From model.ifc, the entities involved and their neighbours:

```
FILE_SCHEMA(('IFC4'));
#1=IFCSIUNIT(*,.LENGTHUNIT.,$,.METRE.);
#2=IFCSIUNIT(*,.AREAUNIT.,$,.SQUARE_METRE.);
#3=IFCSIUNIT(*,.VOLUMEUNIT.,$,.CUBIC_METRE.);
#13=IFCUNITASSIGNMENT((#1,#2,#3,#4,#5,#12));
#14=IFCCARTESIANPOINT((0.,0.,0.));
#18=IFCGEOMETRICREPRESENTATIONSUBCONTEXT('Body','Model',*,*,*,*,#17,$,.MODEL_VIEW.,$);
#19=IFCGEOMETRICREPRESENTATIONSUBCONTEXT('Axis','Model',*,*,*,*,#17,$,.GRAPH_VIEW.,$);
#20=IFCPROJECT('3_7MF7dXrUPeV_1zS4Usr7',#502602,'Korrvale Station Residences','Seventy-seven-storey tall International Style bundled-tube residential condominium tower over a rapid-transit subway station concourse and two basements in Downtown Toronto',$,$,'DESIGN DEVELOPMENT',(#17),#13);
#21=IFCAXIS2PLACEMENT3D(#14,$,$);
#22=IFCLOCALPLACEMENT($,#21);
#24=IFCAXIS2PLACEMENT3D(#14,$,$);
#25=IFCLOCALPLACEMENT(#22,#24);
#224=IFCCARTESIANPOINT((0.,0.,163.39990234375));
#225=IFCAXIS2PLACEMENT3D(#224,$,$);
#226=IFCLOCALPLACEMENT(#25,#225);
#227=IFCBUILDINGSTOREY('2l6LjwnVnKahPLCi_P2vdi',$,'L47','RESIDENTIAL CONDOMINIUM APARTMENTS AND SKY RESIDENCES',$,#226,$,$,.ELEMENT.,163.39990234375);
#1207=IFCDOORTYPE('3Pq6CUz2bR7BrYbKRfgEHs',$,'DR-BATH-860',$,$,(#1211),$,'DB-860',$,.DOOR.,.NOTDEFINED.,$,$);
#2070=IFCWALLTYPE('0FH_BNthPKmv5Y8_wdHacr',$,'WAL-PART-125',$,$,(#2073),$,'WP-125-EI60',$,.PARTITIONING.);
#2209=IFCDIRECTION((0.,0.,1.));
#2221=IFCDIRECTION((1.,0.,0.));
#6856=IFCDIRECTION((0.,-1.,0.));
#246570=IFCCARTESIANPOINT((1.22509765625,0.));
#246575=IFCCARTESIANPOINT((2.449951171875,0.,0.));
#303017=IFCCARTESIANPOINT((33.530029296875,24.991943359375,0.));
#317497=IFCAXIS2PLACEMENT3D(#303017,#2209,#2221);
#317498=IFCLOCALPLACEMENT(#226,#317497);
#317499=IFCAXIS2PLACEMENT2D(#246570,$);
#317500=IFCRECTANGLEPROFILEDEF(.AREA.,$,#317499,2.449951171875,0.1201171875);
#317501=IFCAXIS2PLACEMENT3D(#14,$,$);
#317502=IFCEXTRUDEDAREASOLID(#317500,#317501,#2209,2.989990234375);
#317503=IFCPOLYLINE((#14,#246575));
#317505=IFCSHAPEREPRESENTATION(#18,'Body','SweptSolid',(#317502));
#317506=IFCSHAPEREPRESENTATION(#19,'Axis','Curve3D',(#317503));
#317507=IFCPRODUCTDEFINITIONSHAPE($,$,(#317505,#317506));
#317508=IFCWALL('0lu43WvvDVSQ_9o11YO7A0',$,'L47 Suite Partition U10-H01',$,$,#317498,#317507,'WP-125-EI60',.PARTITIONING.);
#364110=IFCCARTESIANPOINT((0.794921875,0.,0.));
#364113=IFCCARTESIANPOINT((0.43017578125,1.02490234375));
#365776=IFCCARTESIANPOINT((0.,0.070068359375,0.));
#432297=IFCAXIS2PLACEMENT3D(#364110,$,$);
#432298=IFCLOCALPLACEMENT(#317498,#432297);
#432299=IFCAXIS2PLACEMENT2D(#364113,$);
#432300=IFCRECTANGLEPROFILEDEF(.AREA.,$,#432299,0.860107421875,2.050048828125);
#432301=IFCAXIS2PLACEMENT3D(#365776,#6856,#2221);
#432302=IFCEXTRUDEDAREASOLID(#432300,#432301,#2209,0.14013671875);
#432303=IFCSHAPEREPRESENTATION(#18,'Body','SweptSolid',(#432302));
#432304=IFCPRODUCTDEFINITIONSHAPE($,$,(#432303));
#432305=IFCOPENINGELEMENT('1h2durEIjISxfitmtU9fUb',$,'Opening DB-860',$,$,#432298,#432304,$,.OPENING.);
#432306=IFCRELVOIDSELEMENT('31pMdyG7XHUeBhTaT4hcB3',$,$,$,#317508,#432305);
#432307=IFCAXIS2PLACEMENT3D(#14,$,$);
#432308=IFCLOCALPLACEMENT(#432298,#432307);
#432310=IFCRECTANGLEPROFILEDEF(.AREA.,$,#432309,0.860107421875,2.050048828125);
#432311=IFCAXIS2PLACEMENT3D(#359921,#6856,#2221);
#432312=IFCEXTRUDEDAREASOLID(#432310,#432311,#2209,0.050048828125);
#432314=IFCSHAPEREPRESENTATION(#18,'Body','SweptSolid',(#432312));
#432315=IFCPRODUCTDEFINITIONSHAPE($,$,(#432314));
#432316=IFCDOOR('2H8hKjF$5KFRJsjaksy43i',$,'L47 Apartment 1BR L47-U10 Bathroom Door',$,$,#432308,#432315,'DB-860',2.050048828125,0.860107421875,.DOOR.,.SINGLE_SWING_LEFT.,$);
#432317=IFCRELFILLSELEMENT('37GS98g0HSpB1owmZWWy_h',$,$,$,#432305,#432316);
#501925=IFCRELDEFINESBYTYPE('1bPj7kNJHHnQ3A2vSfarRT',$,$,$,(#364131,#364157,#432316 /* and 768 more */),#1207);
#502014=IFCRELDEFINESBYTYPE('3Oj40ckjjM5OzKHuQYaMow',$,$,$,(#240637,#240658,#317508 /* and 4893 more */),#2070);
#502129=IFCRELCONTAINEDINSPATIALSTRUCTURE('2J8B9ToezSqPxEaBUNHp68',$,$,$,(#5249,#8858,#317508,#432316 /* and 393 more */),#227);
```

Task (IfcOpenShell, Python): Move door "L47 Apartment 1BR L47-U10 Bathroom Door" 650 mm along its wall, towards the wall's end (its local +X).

```python
import ifcopenshell
import ifcopenshell.api.geometry
import ifcopenshell.util.placement
import ifcopenshell.util.unit

model = ifcopenshell.open("model.ifc")
unit_scale = ifcopenshell.util.unit.calculate_unit_scale(model)

door = model.by_guid("2H8hKjF$5KFRJsjaksy43i")
opening = door.FillsVoids[0].RelatingOpeningElement
wall = opening.VoidsElements[0].RelatingBuildingElement

wall_matrix = ifcopenshell.util.placement.get_local_placement(wall.ObjectPlacement)
shift = wall_matrix[:3, 0] * 0.65 / unit_scale
before = ifcopenshell.util.placement.get_local_placement(door.ObjectPlacement)[:3, 3].copy()

# The door is placed relative to its opening, so it follows when the opening moves.
matrix = ifcopenshell.util.placement.get_local_placement(opening.ObjectPlacement)
matrix[:3, 3] += shift
ifcopenshell.api.geometry.edit_object_placement(
    model, product=opening, matrix=matrix, is_si=False, should_transform_children=True
)

after = ifcopenshell.util.placement.get_local_placement(door.ObjectPlacement)[:3, 3]
print("door moved by", (after - before).round(3) + 0.0)

model.write("model-out.ifc")
```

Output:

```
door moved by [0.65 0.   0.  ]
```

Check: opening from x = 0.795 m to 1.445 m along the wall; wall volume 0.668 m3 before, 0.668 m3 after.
